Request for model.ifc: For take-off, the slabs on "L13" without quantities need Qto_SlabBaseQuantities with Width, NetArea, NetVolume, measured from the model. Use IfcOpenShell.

First a look at what the model holds.

```python
import ifcopenshell
import ifcopenshell.util.element
import ifcopenshell.util.unit

model = ifcopenshell.open("model.ifc")
print(model.schema)
for unit_type in ("LENGTHUNIT", "AREAUNIT", "VOLUMEUNIT"):
    print(unit_type, ifcopenshell.util.unit.calculate_unit_scale(model, unit_type))
storey = next(s for s in model.by_type("IfcBuildingStorey") if s.Name == "L13")
slabs = [e for e in ifcopenshell.util.element.get_decomposition(storey) if e.is_a("IfcSlab")]
for e in sorted(slabs, key=lambda e: e.id()):
    print(e.id(), e.is_a(), e.Name, list(ifcopenshell.util.element.get_psets(e, qtos_only=True)), sep=" | ")
```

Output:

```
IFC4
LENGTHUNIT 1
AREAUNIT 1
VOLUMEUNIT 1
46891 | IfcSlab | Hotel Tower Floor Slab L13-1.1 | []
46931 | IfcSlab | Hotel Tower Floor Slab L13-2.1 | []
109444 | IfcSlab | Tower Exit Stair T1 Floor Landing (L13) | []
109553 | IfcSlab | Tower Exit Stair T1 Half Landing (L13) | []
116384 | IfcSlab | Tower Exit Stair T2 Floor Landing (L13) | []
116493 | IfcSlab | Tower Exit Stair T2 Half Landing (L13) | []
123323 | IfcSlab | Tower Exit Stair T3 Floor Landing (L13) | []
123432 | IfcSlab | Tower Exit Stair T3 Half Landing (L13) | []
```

```python
import ifcopenshell
import ifcopenshell.api.pset
import ifcopenshell.geom
import ifcopenshell.util.element
import ifcopenshell.util.shape
import ifcopenshell.util.unit

model = ifcopenshell.open("model.ifc")
unit_scale = ifcopenshell.util.unit.calculate_unit_scale(model)
area_scale = ifcopenshell.util.unit.calculate_unit_scale(model, "AREAUNIT")
volume_scale = ifcopenshell.util.unit.calculate_unit_scale(model, "VOLUMEUNIT")
settings = ifcopenshell.geom.settings()

storey = next(s for s in model.by_type("IfcBuildingStorey") if s.Name == "L13")
slabs = [e for e in ifcopenshell.util.element.get_decomposition(storey) if e.is_a("IfcSlab")]

for e in sorted(slabs, key=lambda e: e.id()):
    if ifcopenshell.util.element.get_psets(e, qtos_only=True, should_inherit=False):
        continue
    # Geometry comes back in metres, in the element's own axes.
    shape = ifcopenshell.geom.create_shape(settings, e)
    values = {
        "Width": ifcopenshell.util.shape.get_z(shape.geometry) / unit_scale,
        "NetArea": ifcopenshell.util.shape.get_footprint_area(shape.geometry) / area_scale,
        "NetVolume": ifcopenshell.util.shape.get_volume(shape.geometry) / volume_scale,
    }
    qto = ifcopenshell.api.pset.add_qto(model, product=e, name="Qto_SlabBaseQuantities")
    ifcopenshell.api.pset.edit_qto(model, qto=qto, properties=values)
    print(e.id(), {k: round(v, 3) for k, v in values.items()})

model.write("model_updated.ifc")
```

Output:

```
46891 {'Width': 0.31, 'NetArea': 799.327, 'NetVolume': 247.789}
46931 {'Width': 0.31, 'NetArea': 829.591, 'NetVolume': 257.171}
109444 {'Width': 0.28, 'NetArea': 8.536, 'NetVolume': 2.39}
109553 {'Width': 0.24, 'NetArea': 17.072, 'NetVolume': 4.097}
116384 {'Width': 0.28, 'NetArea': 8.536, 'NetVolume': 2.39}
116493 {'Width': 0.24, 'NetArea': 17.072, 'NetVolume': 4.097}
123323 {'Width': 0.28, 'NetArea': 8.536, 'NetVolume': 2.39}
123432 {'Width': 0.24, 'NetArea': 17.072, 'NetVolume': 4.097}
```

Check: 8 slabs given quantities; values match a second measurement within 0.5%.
